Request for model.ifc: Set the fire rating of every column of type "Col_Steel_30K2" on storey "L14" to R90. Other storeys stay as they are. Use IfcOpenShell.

First a look at what the model holds.

```python
import ifcopenshell
import ifcopenshell.util.element

model = ifcopenshell.open("model.ifc")
print(model.schema)
storey = next(s for s in model.by_type("IfcBuildingStorey") if s.Name == "L14")
columns = [e for e in ifcopenshell.util.element.get_decomposition(storey) if e.is_a("IfcColumn")]
seen = {}
for e in columns:
    element_type = ifcopenshell.util.element.get_type(e)
    key = (element_type.Name if element_type != e and element_type else None, ifcopenshell.util.element.get_pset(e, "Pset_ColumnCommon", "FireRating"))
    seen[key] = seen.get(key, 0) + 1
for (name, value), count in sorted(seen.items(), key=str):
    print(count, "x", name, "|", value)
```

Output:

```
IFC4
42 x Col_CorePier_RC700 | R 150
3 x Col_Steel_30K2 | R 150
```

```python
import ifcopenshell
import ifcopenshell.api.pset
import ifcopenshell.util.element

model = ifcopenshell.open("model.ifc")

storey = next(s for s in model.by_type("IfcBuildingStorey") if s.Name == "L14")
columns = [e for e in ifcopenshell.util.element.get_decomposition(storey) if e.is_a("IfcColumn")]

count = 0
for e in columns:
    element_type = ifcopenshell.util.element.get_type(e)
    if element_type in (None, e) or element_type.Name != "Col_Steel_30K2":
        continue
    # add_pset returns the element's existing set when there is one.
    pset = ifcopenshell.api.pset.add_pset(model, product=e, name="Pset_ColumnCommon")
    ifcopenshell.api.pset.edit_pset(model, pset=pset, properties={"FireRating": "R90"})
    count += 1

print(count, "columns updated")

model.write("model_v2.ifc")
```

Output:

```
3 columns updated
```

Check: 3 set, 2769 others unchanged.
